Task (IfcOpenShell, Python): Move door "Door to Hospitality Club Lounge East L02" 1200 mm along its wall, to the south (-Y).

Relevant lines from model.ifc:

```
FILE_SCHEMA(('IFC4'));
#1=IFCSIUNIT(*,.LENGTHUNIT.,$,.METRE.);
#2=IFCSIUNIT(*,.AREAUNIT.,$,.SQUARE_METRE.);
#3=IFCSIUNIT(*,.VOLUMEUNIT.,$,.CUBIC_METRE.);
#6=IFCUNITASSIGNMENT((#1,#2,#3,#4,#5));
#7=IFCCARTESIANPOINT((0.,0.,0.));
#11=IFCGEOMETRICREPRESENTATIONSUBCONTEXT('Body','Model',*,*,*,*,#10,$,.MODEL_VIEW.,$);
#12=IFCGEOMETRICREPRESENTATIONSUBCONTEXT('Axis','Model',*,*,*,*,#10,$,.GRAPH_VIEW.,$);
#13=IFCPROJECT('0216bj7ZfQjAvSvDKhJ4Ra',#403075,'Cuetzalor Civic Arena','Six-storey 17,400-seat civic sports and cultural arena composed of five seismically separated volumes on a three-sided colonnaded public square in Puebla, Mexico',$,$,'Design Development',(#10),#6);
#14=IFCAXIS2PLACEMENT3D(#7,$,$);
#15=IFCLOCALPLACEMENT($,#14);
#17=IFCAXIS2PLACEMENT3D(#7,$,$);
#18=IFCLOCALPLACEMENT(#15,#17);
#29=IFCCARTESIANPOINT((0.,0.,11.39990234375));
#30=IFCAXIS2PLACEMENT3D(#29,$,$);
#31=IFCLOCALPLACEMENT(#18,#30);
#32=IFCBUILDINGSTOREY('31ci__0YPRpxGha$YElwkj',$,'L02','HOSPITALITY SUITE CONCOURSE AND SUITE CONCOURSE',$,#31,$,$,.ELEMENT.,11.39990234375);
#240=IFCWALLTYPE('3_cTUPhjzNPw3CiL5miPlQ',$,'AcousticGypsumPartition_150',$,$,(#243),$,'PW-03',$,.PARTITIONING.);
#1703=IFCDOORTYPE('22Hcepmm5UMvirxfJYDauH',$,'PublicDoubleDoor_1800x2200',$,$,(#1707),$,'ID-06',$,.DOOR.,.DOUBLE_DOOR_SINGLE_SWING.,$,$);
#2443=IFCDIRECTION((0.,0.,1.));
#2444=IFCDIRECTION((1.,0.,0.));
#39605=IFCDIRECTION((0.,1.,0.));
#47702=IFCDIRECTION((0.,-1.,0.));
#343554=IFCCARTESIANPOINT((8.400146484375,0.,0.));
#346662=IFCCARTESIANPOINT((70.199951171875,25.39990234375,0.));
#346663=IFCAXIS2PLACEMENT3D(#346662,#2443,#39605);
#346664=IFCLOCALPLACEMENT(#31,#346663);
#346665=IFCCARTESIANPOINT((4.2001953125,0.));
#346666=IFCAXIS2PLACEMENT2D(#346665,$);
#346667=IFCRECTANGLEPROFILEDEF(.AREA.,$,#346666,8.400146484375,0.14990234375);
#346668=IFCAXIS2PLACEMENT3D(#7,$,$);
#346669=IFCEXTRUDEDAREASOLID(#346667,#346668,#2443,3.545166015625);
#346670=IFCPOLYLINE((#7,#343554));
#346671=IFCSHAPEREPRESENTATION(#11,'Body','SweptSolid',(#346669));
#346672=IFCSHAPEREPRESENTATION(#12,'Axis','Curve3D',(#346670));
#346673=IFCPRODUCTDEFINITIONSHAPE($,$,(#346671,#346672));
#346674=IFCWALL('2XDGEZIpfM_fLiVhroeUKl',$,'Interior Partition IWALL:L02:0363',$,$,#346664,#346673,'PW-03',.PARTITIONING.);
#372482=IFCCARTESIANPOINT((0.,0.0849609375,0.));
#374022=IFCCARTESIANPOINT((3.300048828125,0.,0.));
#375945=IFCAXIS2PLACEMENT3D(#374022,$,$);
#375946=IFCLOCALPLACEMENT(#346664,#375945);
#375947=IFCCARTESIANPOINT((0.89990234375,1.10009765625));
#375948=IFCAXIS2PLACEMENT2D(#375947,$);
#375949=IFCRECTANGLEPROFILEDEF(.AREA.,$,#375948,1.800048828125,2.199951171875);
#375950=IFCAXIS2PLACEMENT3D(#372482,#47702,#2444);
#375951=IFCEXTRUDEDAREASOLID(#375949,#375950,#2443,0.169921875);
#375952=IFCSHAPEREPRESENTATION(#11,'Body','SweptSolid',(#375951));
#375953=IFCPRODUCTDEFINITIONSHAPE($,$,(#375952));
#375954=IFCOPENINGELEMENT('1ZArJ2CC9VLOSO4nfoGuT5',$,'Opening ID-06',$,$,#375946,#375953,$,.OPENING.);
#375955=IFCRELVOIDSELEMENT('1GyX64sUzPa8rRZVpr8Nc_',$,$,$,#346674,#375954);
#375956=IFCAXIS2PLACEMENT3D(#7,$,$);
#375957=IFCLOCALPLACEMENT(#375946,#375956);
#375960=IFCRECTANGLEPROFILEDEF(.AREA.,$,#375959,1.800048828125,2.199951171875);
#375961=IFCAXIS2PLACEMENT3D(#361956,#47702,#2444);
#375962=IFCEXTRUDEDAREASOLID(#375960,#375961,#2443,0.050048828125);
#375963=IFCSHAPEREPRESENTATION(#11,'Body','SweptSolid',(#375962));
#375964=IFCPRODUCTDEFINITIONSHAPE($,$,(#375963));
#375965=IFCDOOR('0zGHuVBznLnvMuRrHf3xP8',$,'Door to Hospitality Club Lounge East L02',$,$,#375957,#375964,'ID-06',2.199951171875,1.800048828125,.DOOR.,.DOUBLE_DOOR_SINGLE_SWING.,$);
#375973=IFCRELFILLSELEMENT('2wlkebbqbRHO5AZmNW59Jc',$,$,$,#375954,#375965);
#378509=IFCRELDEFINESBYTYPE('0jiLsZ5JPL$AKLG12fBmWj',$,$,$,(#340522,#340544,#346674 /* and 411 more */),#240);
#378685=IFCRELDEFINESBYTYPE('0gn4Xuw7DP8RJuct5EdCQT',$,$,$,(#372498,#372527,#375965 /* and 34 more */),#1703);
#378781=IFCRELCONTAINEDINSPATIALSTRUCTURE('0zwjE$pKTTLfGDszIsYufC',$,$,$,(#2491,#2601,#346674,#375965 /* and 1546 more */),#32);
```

```python
import ifcopenshell
import ifcopenshell.api.geometry
import ifcopenshell.util.placement
import ifcopenshell.util.unit

model = ifcopenshell.open("model.ifc")
unit_scale = ifcopenshell.util.unit.calculate_unit_scale(model)

door = model.by_id(375965)
opening = door.FillsVoids[0].RelatingOpeningElement
wall = opening.VoidsElements[0].RelatingBuildingElement

wall_matrix = ifcopenshell.util.placement.get_local_placement(wall.ObjectPlacement)
shift = wall_matrix[:3, 0] * -1.2 / unit_scale
before = ifcopenshell.util.placement.get_local_placement(door.ObjectPlacement)[:3, 3].copy()

# The door is placed relative to its opening, so it follows when the opening moves.
matrix = ifcopenshell.util.placement.get_local_placement(opening.ObjectPlacement)
matrix[:3, 3] += shift
ifcopenshell.api.geometry.edit_object_placement(
    model, product=opening, matrix=matrix, is_si=False, should_transform_children=True
)

after = ifcopenshell.util.placement.get_local_placement(door.ObjectPlacement)[:3, 3]
print("door moved by", (after - before).round(3) + 0.0)

model.write("model_updated.ifc")
```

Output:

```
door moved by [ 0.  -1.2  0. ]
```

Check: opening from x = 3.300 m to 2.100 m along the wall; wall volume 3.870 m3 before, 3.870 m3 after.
